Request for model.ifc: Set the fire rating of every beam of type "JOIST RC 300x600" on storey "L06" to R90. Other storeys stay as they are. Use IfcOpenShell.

First a look at what the model holds.

```python
import ifcopenshell
import ifcopenshell.util.element

model = ifcopenshell.open("model.ifc")
print(model.schema)
storey = next(s for s in model.by_type("IfcBuildingStorey") if s.Name == "L06")
beams = [e for e in ifcopenshell.util.element.get_decomposition(storey) if e.is_a("IfcBeam")]
seen = {}
for e in beams:
    element_type = ifcopenshell.util.element.get_type(e)
    key = (element_type.Name if element_type != e and element_type else None, ifcopenshell.util.element.get_pset(e, "Pset_BeamCommon", "FireRating"))
    seen[key] = seen.get(key, 0) + 1
for (name, value), count in sorted(seen.items(), key=str):
    print(count, "x", name, "|", value)
```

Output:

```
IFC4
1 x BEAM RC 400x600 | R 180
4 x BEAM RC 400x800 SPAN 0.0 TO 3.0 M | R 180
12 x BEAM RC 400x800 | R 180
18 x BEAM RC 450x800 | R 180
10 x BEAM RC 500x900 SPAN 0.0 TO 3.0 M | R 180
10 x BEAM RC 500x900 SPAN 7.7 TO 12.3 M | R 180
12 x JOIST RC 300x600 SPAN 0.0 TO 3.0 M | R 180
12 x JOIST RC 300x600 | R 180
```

```python
import ifcopenshell
import ifcopenshell.api.pset
import ifcopenshell.util.element

model = ifcopenshell.open("model.ifc")

storey = next(s for s in model.by_type("IfcBuildingStorey") if s.Name == "L06")
beams = [e for e in ifcopenshell.util.element.get_decomposition(storey) if e.is_a("IfcBeam")]

count = 0
for e in beams:
    element_type = ifcopenshell.util.element.get_type(e)
    if element_type in (None, e) or element_type.Name != "JOIST RC 300x600":
        continue
    # add_pset returns the element's existing set when there is one.
    pset = ifcopenshell.api.pset.add_pset(model, product=e, name="Pset_BeamCommon")
    ifcopenshell.api.pset.edit_pset(model, pset=pset, properties={"FireRating": "R90"})
    count += 1

print(count, "beams updated")

model.write("model_edited.ifc")
```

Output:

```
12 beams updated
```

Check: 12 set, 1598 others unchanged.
